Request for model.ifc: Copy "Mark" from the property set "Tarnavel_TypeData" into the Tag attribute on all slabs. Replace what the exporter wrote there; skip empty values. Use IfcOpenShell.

First a look at what the model holds.

```python
import ifcopenshell
import ifcopenshell.util.element

model = ifcopenshell.open("model.ifc")
print(model.schema)
slabs = model.by_type("IfcSlab")
print(len(slabs), "slabs")
for e in slabs[:8]:
    source = ifcopenshell.util.element.get_pset(e, "Tarnavel_TypeData", "Mark")
    target = e.Tag
    print(e.id(), repr(source), repr(target), sep=" | ")
```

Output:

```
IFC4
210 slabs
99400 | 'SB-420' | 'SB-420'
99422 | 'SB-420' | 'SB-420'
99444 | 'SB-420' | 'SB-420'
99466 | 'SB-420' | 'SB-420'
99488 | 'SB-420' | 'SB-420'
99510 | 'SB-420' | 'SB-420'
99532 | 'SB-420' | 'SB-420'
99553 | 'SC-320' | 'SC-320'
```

```python
import ifcopenshell
import ifcopenshell.util.element

model = ifcopenshell.open("model.ifc")

count = 0
for e in model.by_type("IfcSlab"):
    value = ifcopenshell.util.element.get_pset(e, "Tarnavel_TypeData", "Mark")
    current = e.Tag
    if not value or not value.strip() or current == value:
        continue
    e.Tag = value
    count += 1

print(count, "slabs updated")

model.write("model_v2.ifc")
```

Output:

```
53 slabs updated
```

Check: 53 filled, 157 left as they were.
